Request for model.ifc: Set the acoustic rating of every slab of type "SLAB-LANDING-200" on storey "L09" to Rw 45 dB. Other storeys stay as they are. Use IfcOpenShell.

First a look at what the model holds.

```python
import ifcopenshell
import ifcopenshell.util.element

model = ifcopenshell.open("model.ifc")
print(model.schema)
storey = next(s for s in model.by_type("IfcBuildingStorey") if s.Name == "L09")
slabs = [e for e in ifcopenshell.util.element.get_decomposition(storey) if e.is_a("IfcSlab")]
seen = {}
for e in slabs:
    element_type = ifcopenshell.util.element.get_type(e)
    key = (element_type.Name if element_type != e and element_type else None, ifcopenshell.util.element.get_pset(e, "Pset_SlabCommon", "AcousticRating"))
    seen[key] = seen.get(key, 0) + 1
for (name, value), count in sorted(seen.items(), key=str):
    print(count, "x", name, "|", value)
```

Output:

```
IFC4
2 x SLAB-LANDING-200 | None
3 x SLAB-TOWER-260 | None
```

```python
import ifcopenshell
import ifcopenshell.api.pset
import ifcopenshell.util.element

model = ifcopenshell.open("model.ifc")

storey = next(s for s in model.by_type("IfcBuildingStorey") if s.Name == "L09")
slabs = [e for e in ifcopenshell.util.element.get_decomposition(storey) if e.is_a("IfcSlab")]

count = 0
for e in slabs:
    element_type = ifcopenshell.util.element.get_type(e)
    if element_type in (None, e) or element_type.Name != "SLAB-LANDING-200":
        continue
    found = ifcopenshell.util.element.get_pset(e, "Pset_SlabCommon", should_inherit=False)
    if found:
        pset = model.by_id(found["id"])
        if len(ifcopenshell.util.element.get_elements_by_pset(pset)) > 1:
            pset = ifcopenshell.api.pset.unshare_pset(model, products=[e], pset=pset)[0]
    else:
        pset = ifcopenshell.api.pset.add_pset(model, product=e, name="Pset_SlabCommon")
    ifcopenshell.api.pset.edit_pset(model, pset=pset, properties={"AcousticRating": "Rw 45 dB"})
    count += 1

print(count, "slabs updated")

model.write("model_updated.ifc")
```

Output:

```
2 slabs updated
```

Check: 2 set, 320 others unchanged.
